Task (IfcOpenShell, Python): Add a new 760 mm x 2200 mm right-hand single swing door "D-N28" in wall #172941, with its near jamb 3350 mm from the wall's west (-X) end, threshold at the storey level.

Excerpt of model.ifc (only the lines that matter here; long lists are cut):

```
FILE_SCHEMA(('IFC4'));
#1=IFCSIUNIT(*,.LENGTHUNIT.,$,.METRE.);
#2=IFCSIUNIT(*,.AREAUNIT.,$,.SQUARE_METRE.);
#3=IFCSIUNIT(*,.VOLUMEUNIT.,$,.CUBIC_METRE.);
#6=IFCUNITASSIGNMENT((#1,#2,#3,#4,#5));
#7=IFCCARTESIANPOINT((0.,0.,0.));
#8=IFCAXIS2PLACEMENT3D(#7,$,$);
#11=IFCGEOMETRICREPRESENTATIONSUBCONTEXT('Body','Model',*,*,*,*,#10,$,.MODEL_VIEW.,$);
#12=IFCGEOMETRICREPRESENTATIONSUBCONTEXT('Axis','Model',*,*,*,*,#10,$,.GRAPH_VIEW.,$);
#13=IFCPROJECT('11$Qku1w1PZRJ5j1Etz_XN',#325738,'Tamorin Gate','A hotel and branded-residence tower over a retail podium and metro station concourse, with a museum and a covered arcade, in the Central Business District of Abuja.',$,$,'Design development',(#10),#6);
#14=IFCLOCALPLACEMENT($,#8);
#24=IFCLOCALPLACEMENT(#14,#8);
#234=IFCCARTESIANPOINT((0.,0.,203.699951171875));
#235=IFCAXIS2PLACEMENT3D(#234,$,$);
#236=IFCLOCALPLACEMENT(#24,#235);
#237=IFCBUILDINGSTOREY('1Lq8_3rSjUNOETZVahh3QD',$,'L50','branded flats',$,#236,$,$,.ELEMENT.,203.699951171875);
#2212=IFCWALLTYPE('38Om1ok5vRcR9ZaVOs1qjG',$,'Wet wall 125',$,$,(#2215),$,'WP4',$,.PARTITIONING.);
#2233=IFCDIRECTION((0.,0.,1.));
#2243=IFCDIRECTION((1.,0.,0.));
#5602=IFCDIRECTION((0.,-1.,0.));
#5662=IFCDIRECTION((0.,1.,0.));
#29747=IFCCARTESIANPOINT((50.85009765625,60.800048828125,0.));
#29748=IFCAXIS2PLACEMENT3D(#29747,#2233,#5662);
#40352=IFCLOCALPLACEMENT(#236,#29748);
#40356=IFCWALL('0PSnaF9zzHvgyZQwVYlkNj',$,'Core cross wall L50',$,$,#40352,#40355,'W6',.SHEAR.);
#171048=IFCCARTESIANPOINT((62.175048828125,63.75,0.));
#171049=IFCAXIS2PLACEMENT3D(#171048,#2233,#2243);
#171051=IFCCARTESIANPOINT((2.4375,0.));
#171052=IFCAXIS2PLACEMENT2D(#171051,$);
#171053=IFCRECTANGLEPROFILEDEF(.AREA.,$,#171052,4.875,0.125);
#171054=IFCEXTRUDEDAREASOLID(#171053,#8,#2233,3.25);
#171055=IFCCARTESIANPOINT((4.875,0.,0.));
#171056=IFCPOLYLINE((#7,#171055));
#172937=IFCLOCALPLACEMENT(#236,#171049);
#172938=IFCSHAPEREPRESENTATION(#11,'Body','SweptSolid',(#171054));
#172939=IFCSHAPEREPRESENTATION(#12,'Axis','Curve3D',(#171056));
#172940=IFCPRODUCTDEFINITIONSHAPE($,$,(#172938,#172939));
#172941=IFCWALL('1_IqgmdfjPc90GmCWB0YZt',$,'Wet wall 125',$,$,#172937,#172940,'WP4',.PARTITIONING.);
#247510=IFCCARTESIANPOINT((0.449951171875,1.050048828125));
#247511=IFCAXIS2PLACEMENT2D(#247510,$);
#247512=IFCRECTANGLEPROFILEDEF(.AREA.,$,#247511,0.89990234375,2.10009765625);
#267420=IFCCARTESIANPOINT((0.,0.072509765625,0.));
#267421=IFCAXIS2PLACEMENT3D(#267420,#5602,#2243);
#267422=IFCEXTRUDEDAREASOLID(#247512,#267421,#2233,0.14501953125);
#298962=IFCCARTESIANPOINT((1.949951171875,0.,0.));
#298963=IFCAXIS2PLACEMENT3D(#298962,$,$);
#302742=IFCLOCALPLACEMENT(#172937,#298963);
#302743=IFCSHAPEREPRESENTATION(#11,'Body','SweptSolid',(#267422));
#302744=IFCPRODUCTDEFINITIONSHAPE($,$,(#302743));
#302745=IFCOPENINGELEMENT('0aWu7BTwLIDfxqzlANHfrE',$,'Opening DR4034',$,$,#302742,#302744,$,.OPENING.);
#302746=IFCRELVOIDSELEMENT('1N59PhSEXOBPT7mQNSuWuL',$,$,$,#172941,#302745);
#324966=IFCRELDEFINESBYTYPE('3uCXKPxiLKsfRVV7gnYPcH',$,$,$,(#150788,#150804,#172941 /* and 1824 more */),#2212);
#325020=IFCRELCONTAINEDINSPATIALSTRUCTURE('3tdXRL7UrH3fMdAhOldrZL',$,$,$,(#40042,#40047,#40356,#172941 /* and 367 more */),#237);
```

```python
import numpy as np
import ifcopenshell
import ifcopenshell.api.feature
import ifcopenshell.api.geometry
import ifcopenshell.api.root
import ifcopenshell.api.spatial
import ifcopenshell.geom
import ifcopenshell.util.element
import ifcopenshell.util.placement
import ifcopenshell.util.representation
import ifcopenshell.util.shape
import ifcopenshell.util.unit

model = ifcopenshell.open("model.ifc")
unit_scale = ifcopenshell.util.unit.calculate_unit_scale(model)
settings = ifcopenshell.geom.settings()


def volume(element):
    """Net volume in cubic metres, openings subtracted."""
    shape = ifcopenshell.geom.create_shape(settings, element)
    return ifcopenshell.util.shape.get_volume(shape.geometry)


wall = model.by_guid("1_IqgmdfjPc90GmCWB0YZt")
storey = ifcopenshell.util.element.get_container(wall, ifc_class="IfcBuildingStorey")
context = ifcopenshell.util.representation.get_context(model, "Model", "Body", "MODEL_VIEW")
before = volume(wall)

width, height, from_end, sill = 0.76, 2.2, 3.35, 0.0  # metres

# The wall runs along its own X axis, and the end named is its -X end.
wall_shape = ifcopenshell.geom.create_shape(settings, wall)
x, y, z = ifcopenshell.util.shape.get_vertices(wall_shape.geometry).T
start = x.min() + from_end
face, thickness = float(y.min()), float(y.max() - y.min())
wall_matrix = ifcopenshell.util.placement.get_local_placement(wall.ObjectPlacement)
level = ifcopenshell.util.placement.get_local_placement(storey.ObjectPlacement)[2, 3]


def in_wall(x, y):
    """Placement at x, y metres in the wall's axes, at sill height."""
    matrix = wall_matrix.copy()
    matrix[:, 3] = wall_matrix @ np.array([x / unit_scale, y / unit_scale, 0.0, 1.0])
    matrix[2, 3] = level + sill / unit_scale
    return matrix


# Opening: a box that overshoots both wall faces by 50 mm.
opening = ifcopenshell.api.root.create_entity(model, ifc_class="IfcOpeningElement", predefined_type="OPENING")
box = ifcopenshell.api.geometry.add_wall_representation(
    model, context=context, length=width, height=height, thickness=thickness + 0.1
)
ifcopenshell.api.geometry.assign_representation(model, product=opening, representation=box)
ifcopenshell.api.geometry.edit_object_placement(model, product=opening, matrix=in_wall(start, face - 0.05), is_si=False)
ifcopenshell.api.feature.add_feature(model, feature=opening, element=wall)

door = ifcopenshell.api.root.create_entity(model, ifc_class="IfcDoor", name="D-N28", predefined_type="DOOR")
door.OverallWidth, door.OverallHeight = width / unit_scale, height / unit_scale
door.OperationType = "SINGLE_SWING_RIGHT"
body = ifcopenshell.api.geometry.add_door_representation(
    model,
    context=context,
    overall_width=door.OverallWidth,
    overall_height=door.OverallHeight,
    operation_type="SINGLE_SWING_RIGHT",
    lining_properties={"LiningDepth": thickness / unit_scale, "ThresholdDepth": thickness / unit_scale},
)
ifcopenshell.api.geometry.assign_representation(model, product=door, representation=body)
ifcopenshell.api.spatial.assign_container(model, products=[door], relating_structure=storey)
ifcopenshell.api.feature.add_filling(model, opening=opening, element=door)

# The lining spans the wall, so the door starts at the wall face.
ifcopenshell.api.geometry.edit_object_placement(model, product=door, matrix=in_wall(start, face), is_si=False)

after = volume(wall)

print(f"wall volume {before:.3f} -> {after:.3f} m3")

model.write("model-out.ifc")
```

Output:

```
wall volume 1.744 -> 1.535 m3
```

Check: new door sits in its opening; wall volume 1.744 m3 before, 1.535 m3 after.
